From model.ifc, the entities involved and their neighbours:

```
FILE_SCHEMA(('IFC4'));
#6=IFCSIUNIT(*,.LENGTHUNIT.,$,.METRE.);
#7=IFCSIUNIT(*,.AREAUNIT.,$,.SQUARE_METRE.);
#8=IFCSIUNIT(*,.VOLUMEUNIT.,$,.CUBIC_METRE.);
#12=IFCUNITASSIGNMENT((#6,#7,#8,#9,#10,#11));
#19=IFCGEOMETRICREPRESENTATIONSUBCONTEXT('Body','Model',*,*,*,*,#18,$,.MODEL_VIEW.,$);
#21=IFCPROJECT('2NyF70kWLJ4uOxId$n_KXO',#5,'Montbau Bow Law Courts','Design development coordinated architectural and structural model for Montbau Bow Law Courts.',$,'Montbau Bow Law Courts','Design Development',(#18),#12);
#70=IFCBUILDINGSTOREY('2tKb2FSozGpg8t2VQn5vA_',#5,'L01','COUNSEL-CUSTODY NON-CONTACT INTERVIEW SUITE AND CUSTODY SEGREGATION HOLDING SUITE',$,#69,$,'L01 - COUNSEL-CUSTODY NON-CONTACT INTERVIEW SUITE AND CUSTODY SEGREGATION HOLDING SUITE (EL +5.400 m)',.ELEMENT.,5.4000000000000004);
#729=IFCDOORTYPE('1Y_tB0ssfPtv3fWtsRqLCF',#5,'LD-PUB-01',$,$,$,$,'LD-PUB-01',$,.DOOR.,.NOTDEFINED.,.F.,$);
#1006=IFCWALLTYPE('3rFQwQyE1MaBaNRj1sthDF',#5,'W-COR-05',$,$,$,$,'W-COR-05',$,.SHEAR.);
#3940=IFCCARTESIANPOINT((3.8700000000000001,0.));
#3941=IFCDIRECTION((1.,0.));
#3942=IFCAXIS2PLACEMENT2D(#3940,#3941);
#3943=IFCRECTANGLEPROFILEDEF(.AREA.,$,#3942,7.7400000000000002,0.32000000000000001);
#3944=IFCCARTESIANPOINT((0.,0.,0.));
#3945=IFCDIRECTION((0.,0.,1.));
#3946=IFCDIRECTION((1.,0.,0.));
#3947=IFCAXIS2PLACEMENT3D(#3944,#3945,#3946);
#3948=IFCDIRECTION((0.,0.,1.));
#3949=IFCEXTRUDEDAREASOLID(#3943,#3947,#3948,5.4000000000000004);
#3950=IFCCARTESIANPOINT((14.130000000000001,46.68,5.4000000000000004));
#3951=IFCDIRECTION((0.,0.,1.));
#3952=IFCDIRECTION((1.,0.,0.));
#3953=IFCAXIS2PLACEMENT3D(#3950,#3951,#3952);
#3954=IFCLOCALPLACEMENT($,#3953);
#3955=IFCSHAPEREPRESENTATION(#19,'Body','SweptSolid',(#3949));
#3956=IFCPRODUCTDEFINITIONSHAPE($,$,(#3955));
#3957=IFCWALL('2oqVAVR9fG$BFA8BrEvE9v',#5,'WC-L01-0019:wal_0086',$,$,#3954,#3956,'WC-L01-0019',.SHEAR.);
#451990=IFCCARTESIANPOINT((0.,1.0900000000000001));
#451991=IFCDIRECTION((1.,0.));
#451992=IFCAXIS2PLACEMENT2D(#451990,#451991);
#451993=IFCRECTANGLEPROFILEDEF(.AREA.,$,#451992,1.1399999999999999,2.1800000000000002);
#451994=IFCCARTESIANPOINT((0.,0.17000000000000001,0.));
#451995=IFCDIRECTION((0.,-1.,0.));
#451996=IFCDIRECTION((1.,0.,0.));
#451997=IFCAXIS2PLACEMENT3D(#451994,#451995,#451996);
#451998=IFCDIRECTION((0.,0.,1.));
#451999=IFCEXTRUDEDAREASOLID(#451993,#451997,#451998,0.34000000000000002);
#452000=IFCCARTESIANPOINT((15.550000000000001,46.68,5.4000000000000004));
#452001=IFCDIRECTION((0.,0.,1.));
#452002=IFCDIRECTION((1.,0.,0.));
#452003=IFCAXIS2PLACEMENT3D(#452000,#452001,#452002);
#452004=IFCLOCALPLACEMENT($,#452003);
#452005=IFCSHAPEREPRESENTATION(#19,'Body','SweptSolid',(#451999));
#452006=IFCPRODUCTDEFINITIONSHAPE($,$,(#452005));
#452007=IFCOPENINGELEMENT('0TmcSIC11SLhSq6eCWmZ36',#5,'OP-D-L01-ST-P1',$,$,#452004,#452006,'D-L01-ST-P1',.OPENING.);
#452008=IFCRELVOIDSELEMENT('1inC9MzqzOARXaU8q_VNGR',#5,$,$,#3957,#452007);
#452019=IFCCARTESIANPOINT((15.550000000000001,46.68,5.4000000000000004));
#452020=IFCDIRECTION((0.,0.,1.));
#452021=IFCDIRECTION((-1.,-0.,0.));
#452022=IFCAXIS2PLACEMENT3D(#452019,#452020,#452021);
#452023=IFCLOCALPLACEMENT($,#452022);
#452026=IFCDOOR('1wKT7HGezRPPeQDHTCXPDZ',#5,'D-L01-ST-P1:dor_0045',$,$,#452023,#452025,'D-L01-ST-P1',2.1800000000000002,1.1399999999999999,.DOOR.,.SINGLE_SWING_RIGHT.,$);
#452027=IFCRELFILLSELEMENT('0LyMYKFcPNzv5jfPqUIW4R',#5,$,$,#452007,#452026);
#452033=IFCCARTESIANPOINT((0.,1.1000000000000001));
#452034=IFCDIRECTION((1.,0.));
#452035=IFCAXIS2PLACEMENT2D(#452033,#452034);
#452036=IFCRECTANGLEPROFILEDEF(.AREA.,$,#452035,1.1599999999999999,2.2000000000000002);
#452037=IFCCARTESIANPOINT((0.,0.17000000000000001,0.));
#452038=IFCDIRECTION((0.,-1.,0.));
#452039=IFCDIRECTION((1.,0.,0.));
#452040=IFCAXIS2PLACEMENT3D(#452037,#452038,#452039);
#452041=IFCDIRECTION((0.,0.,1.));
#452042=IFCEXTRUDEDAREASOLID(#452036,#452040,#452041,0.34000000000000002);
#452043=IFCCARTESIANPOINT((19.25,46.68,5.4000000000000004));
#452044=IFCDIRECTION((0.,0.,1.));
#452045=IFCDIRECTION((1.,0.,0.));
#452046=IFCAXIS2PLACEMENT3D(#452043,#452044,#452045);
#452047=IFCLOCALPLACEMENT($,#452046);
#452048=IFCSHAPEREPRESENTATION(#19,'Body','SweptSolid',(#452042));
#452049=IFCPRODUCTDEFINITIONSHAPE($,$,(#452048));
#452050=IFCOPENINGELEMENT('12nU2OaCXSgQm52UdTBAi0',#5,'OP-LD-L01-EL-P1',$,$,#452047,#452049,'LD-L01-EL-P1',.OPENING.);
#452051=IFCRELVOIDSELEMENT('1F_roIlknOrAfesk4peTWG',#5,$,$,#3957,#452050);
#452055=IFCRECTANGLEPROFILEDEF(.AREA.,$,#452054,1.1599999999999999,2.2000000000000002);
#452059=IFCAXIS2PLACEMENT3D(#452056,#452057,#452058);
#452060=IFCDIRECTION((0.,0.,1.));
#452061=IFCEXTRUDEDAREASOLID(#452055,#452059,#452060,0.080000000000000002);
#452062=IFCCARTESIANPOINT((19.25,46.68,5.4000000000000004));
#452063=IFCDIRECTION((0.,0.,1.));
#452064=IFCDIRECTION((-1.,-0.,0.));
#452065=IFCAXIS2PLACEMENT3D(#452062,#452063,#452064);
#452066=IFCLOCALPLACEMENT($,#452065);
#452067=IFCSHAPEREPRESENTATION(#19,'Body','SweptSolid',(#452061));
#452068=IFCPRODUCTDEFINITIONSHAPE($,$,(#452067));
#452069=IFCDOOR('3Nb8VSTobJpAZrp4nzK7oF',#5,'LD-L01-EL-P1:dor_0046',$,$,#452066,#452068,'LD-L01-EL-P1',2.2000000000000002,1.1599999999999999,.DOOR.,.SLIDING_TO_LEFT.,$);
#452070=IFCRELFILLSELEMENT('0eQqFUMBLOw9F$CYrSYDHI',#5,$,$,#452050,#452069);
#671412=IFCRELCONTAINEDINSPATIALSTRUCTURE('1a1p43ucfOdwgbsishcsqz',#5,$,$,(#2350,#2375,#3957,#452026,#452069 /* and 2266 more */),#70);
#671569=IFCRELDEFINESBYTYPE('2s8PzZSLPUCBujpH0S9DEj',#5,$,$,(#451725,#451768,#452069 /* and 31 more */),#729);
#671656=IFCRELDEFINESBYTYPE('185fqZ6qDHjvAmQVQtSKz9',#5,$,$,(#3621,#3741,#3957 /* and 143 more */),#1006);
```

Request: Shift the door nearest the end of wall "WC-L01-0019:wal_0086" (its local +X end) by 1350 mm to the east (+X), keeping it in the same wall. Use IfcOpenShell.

```python
import ifcopenshell
import ifcopenshell.api.geometry
import ifcopenshell.util.placement

model = ifcopenshell.open("model.ifc")

door = model.by_guid("3Nb8VSTobJpAZrp4nzK7oF")
opening = door.FillsVoids[0].RelatingOpeningElement
wall = opening.VoidsElements[0].RelatingBuildingElement

wall_matrix = ifcopenshell.util.placement.get_local_placement(wall.ObjectPlacement)
shift = wall_matrix[:3, 0] * 1.35
before = ifcopenshell.util.placement.get_local_placement(door.ObjectPlacement)[:3, 3].copy()

# The door is not placed relative to its opening, so move both.
for product in (opening, door):
    matrix = ifcopenshell.util.placement.get_local_placement(product.ObjectPlacement)
    matrix[:3, 3] += shift
    ifcopenshell.api.geometry.edit_object_placement(model, product=product, matrix=matrix, is_si=False)

after = ifcopenshell.util.placement.get_local_placement(door.ObjectPlacement)[:3, 3]
print("door moved by", (after - before).round(3) + 0.0)

model.write("model-out.ifc")
```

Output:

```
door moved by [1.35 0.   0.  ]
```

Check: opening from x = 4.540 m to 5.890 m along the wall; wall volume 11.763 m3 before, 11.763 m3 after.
